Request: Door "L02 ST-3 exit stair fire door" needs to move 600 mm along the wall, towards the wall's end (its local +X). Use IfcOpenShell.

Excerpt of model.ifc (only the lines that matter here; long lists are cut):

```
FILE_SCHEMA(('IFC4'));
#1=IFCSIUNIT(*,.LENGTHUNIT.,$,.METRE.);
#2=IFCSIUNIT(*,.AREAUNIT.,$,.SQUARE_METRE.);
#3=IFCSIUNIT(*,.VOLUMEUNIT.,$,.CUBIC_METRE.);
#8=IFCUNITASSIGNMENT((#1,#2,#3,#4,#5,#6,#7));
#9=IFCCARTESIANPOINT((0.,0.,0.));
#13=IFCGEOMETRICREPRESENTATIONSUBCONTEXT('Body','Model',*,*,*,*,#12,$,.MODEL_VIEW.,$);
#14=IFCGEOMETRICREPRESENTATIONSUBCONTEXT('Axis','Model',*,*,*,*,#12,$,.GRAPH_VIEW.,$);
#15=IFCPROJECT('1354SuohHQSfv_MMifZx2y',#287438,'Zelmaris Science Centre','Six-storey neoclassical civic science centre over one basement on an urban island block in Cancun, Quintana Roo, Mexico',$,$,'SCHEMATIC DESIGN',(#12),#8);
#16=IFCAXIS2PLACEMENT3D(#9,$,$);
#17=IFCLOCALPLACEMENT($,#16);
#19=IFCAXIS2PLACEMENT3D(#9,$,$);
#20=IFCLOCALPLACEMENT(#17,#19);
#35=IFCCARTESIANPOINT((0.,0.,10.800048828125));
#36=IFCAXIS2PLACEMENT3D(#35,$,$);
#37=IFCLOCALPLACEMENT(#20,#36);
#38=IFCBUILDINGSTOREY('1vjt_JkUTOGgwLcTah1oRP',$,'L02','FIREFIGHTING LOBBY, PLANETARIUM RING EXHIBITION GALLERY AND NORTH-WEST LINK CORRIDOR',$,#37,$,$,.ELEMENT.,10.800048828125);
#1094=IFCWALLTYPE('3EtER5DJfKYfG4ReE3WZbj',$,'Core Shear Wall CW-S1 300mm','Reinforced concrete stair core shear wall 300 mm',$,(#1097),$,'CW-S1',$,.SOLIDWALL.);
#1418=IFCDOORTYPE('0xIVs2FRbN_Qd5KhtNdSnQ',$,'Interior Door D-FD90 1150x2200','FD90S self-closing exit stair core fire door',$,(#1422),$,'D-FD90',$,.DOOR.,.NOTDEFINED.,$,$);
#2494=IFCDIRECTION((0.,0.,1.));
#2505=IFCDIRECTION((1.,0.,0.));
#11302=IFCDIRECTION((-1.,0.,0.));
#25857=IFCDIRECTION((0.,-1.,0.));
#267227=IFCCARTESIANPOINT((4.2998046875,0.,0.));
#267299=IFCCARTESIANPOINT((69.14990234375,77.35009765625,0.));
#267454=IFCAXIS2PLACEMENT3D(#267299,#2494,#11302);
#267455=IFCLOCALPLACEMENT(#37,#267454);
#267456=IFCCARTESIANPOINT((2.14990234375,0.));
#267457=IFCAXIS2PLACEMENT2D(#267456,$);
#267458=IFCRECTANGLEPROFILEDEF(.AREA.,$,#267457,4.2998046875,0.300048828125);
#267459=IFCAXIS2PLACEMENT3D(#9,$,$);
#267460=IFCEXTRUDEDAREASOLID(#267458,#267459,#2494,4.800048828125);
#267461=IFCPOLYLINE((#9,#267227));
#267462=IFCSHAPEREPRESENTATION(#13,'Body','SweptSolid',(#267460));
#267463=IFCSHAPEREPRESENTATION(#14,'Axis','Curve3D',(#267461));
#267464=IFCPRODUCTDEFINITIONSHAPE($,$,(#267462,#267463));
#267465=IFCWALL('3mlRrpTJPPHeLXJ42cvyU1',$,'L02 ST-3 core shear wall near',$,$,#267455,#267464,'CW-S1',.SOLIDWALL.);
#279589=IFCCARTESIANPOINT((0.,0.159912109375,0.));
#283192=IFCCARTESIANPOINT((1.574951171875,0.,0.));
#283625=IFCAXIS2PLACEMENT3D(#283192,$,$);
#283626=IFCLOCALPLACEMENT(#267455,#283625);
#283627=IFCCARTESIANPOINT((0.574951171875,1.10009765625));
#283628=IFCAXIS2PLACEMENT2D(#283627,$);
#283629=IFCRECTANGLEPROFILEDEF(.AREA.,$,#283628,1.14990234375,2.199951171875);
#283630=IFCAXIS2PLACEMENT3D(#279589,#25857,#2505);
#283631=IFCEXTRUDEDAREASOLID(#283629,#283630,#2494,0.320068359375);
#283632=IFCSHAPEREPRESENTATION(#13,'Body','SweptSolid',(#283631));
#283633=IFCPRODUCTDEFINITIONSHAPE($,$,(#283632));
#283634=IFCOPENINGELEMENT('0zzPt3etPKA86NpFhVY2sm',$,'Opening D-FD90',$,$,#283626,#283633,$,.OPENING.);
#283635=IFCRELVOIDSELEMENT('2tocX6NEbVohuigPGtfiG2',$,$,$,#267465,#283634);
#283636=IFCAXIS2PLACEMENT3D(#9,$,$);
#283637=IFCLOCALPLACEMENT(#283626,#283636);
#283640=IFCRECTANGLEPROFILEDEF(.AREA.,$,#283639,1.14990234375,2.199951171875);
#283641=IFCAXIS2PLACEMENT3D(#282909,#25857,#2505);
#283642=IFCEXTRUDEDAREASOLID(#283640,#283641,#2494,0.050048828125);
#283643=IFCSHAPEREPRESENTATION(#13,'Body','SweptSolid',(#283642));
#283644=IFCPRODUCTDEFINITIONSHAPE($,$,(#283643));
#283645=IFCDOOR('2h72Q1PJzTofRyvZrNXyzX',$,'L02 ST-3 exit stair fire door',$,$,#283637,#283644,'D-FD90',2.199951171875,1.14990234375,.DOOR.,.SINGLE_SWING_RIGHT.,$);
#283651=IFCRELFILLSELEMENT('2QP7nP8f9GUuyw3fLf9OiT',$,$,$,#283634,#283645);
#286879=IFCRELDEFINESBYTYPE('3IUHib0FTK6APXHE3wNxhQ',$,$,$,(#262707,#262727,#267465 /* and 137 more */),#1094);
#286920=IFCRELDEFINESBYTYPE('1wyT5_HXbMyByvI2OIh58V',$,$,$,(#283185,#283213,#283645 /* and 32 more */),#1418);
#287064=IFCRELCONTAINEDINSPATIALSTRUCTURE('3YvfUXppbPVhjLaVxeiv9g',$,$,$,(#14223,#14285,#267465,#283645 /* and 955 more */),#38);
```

```python
import ifcopenshell
import ifcopenshell.api.geometry
import ifcopenshell.util.placement
import ifcopenshell.util.unit

model = ifcopenshell.open("model.ifc")
unit_scale = ifcopenshell.util.unit.calculate_unit_scale(model)

door = model.by_guid("2h72Q1PJzTofRyvZrNXyzX")
opening = door.FillsVoids[0].RelatingOpeningElement
wall = opening.VoidsElements[0].RelatingBuildingElement

wall_matrix = ifcopenshell.util.placement.get_local_placement(wall.ObjectPlacement)
shift = wall_matrix[:3, 0] * 0.6 / unit_scale
before = ifcopenshell.util.placement.get_local_placement(door.ObjectPlacement)[:3, 3].copy()

# The door is placed relative to its opening, so it follows when the opening moves.
matrix = ifcopenshell.util.placement.get_local_placement(opening.ObjectPlacement)
matrix[:3, 3] += shift
ifcopenshell.api.geometry.edit_object_placement(
    model, product=opening, matrix=matrix, is_si=False, should_transform_children=True
)

after = ifcopenshell.util.placement.get_local_placement(door.ObjectPlacement)[:3, 3]
print("door moved by", (after - before).round(3) + 0.0)

model.write("model-out.ifc")
```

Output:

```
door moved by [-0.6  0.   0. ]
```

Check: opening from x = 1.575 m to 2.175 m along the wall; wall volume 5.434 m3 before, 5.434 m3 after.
